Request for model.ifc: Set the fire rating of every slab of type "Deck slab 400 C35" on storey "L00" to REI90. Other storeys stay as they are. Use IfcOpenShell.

First a look at what the model holds.

```python
import ifcopenshell
import ifcopenshell.util.element

model = ifcopenshell.open("model.ifc")
print(model.schema)
storey = next(s for s in model.by_type("IfcBuildingStorey") if s.Name == "L00")
slabs = [e for e in ifcopenshell.util.element.get_decomposition(storey) if e.is_a("IfcSlab")]
seen = {}
for e in slabs:
    element_type = ifcopenshell.util.element.get_type(e)
    key = (element_type.Name if element_type != e and element_type else None, ifcopenshell.util.element.get_pset(e, "Pset_SlabCommon", "FireRating"))
    seen[key] = seen.get(key, 0) + 1
for (name, value), count in sorted(seen.items(), key=str):
    print(count, "x", name, "|", value)
```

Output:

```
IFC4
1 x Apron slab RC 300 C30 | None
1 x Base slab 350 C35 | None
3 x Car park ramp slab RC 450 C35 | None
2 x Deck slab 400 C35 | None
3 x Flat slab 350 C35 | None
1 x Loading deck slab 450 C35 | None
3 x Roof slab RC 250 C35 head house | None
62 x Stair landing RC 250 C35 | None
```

```python
import ifcopenshell
import ifcopenshell.api.pset
import ifcopenshell.util.element

model = ifcopenshell.open("model.ifc")

storey = next(s for s in model.by_type("IfcBuildingStorey") if s.Name == "L00")
slabs = [e for e in ifcopenshell.util.element.get_decomposition(storey) if e.is_a("IfcSlab")]

count = 0
for e in slabs:
    element_type = ifcopenshell.util.element.get_type(e)
    if element_type in (None, e) or element_type.Name != "Deck slab 400 C35":
        continue
    # add_pset returns the element's existing set when there is one.
    pset = ifcopenshell.api.pset.add_pset(model, product=e, name="Pset_SlabCommon")
    ifcopenshell.api.pset.edit_pset(model, pset=pset, properties={"FireRating": "REI90"})
    count += 1

print(count, "slabs updated")

model.write("model_v2.ifc")
```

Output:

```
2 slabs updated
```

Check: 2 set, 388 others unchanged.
